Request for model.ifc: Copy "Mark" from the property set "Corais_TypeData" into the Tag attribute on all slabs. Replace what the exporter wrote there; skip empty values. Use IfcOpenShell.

First a look at what the model holds.

```python
import ifcopenshell
import ifcopenshell.util.element

model = ifcopenshell.open("model.ifc")
print(model.schema)
slabs = model.by_type("IfcSlab")
print(len(slabs), "slabs")
for e in slabs[:8]:
    source = ifcopenshell.util.element.get_pset(e, "Corais_TypeData", "Mark")
    target = e.Tag
    print(e.id(), repr(source), repr(target), sep=" | ")
```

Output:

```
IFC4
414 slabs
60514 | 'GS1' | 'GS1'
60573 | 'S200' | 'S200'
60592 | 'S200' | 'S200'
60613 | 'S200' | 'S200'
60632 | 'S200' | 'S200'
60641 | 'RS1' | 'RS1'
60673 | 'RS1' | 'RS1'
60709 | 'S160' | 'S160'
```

```python
import ifcopenshell
import ifcopenshell.util.element

model = ifcopenshell.open("model.ifc")

count = 0
for e in model.by_type("IfcSlab"):
    value = ifcopenshell.util.element.get_pset(e, "Corais_TypeData", "Mark")
    current = e.Tag
    if not value or not value.strip() or current == value:
        continue
    e.Tag = value
    count += 1

print(count, "slabs updated")

model.write("model_rev.ifc")
```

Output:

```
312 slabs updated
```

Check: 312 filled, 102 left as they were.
